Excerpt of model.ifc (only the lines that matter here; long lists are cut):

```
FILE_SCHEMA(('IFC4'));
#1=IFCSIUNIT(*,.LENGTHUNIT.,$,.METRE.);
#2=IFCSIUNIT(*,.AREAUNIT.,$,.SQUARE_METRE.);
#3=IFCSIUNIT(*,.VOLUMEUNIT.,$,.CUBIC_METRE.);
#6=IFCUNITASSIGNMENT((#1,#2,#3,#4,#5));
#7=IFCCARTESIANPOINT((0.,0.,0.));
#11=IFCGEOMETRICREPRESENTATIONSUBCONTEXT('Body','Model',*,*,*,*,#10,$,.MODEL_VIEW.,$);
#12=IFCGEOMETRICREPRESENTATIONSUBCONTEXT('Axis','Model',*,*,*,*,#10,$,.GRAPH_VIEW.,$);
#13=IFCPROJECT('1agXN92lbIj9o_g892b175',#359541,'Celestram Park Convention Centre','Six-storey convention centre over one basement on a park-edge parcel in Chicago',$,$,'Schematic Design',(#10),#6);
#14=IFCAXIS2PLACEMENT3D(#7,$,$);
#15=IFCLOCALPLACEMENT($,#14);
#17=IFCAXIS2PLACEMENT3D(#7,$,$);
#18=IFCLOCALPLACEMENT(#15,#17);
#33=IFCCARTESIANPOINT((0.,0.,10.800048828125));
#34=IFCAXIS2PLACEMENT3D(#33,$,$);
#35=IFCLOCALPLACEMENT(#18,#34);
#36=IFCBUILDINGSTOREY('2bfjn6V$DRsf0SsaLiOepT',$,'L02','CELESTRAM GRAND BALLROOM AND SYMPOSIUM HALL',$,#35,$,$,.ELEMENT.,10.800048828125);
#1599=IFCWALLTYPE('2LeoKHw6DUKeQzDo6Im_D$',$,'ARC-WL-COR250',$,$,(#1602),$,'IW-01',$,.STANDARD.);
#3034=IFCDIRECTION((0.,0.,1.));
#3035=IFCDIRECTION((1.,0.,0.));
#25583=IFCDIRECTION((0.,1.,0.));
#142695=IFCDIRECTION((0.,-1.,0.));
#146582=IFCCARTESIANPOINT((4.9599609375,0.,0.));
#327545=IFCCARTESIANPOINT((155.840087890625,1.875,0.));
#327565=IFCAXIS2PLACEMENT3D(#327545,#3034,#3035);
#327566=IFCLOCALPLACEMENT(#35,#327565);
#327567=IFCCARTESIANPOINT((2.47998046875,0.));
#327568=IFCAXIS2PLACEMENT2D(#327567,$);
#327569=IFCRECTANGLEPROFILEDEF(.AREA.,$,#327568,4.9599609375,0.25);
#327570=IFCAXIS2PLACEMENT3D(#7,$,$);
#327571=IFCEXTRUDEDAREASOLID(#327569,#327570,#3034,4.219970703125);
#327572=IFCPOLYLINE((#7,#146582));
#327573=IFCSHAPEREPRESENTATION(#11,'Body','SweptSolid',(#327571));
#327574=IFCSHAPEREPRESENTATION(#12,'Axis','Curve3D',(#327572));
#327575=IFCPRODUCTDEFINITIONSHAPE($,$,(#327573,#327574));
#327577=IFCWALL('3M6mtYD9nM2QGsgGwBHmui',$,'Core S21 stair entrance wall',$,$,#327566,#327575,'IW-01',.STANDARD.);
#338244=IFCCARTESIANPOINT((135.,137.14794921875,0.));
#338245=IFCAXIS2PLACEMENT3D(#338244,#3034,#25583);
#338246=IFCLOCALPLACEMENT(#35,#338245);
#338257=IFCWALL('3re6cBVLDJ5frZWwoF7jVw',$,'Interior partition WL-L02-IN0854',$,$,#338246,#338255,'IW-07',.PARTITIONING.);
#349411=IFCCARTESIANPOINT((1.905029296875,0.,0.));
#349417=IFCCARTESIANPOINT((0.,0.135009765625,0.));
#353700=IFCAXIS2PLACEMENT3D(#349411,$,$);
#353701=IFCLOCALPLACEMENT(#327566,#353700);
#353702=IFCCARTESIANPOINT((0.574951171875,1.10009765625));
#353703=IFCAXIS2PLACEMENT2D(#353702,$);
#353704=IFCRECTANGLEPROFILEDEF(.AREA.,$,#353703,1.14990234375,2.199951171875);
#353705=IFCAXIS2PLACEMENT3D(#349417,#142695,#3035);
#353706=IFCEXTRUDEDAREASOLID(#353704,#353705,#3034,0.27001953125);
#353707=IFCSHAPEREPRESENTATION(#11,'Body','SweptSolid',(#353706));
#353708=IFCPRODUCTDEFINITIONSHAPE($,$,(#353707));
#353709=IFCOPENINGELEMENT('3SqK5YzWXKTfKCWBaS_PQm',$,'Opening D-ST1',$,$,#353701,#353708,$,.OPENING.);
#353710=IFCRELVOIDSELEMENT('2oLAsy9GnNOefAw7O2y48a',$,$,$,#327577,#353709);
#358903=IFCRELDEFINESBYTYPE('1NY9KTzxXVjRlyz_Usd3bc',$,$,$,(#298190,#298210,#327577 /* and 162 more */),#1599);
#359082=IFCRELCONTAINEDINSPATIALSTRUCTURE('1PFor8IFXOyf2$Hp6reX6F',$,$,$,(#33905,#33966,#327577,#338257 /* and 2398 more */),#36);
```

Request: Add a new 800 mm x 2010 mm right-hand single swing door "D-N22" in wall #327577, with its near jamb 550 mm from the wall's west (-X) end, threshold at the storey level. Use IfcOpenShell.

```python
import numpy as np
import ifcopenshell
import ifcopenshell.api.feature
import ifcopenshell.api.geometry
import ifcopenshell.api.root
import ifcopenshell.api.spatial
import ifcopenshell.geom
import ifcopenshell.util.element
import ifcopenshell.util.placement
import ifcopenshell.util.representation
import ifcopenshell.util.shape
import ifcopenshell.util.unit

model = ifcopenshell.open("model.ifc")
unit_scale = ifcopenshell.util.unit.calculate_unit_scale(model)
settings = ifcopenshell.geom.settings()


def volume(element):
    """Net volume in cubic metres, openings subtracted."""
    shape = ifcopenshell.geom.create_shape(settings, element)
    return ifcopenshell.util.shape.get_volume(shape.geometry)


wall = model.by_guid("3M6mtYD9nM2QGsgGwBHmui")
storey = ifcopenshell.util.element.get_container(wall, ifc_class="IfcBuildingStorey")
context = ifcopenshell.util.representation.get_context(model, "Model", "Body", "MODEL_VIEW")
before = volume(wall)

width, height, from_end, sill = 0.8, 2.01, 0.55, 0.0  # metres

# The wall runs along its own X axis, and the end named is its -X end.
wall_shape = ifcopenshell.geom.create_shape(settings, wall)
x, y, z = ifcopenshell.util.shape.get_vertices(wall_shape.geometry).T
start = x.min() + from_end
face, thickness = float(y.min()), float(y.max() - y.min())
wall_matrix = ifcopenshell.util.placement.get_local_placement(wall.ObjectPlacement)
level = ifcopenshell.util.placement.get_local_placement(storey.ObjectPlacement)[2, 3]


def in_wall(x, y):
    """Placement at x, y metres in the wall's axes, at sill height."""
    matrix = wall_matrix.copy()
    matrix[:, 3] = wall_matrix @ np.array([x / unit_scale, y / unit_scale, 0.0, 1.0])
    matrix[2, 3] = level + sill / unit_scale
    return matrix


# Opening: a box that overshoots both wall faces by 50 mm.
opening = ifcopenshell.api.root.create_entity(model, ifc_class="IfcOpeningElement", predefined_type="OPENING")
box = ifcopenshell.api.geometry.add_wall_representation(
    model, context=context, length=width, height=height, thickness=thickness + 0.1
)
ifcopenshell.api.geometry.assign_representation(model, product=opening, representation=box)
ifcopenshell.api.geometry.edit_object_placement(model, product=opening, matrix=in_wall(start, face - 0.05), is_si=False)
ifcopenshell.api.feature.add_feature(model, feature=opening, element=wall)

door = ifcopenshell.api.root.create_entity(model, ifc_class="IfcDoor", name="D-N22", predefined_type="DOOR")
door.OverallWidth, door.OverallHeight = width / unit_scale, height / unit_scale
door.OperationType = "SINGLE_SWING_RIGHT"
body = ifcopenshell.api.geometry.add_door_representation(
    model,
    context=context,
    overall_width=door.OverallWidth,
    overall_height=door.OverallHeight,
    operation_type="SINGLE_SWING_RIGHT",
    lining_properties={"LiningDepth": thickness / unit_scale, "ThresholdDepth": thickness / unit_scale},
)
ifcopenshell.api.geometry.assign_representation(model, product=door, representation=body)
ifcopenshell.api.spatial.assign_container(model, products=[door], relating_structure=storey)
ifcopenshell.api.feature.add_filling(model, opening=opening, element=door)

# The lining spans the wall, so the door starts at the wall face.
ifcopenshell.api.geometry.edit_object_placement(model, product=door, matrix=in_wall(start, face), is_si=False)

after = volume(wall)

print(f"wall volume {before:.3f} -> {after:.3f} m3")

model.write("model_v2.ifc")
```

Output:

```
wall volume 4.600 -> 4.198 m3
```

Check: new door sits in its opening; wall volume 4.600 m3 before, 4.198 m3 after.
